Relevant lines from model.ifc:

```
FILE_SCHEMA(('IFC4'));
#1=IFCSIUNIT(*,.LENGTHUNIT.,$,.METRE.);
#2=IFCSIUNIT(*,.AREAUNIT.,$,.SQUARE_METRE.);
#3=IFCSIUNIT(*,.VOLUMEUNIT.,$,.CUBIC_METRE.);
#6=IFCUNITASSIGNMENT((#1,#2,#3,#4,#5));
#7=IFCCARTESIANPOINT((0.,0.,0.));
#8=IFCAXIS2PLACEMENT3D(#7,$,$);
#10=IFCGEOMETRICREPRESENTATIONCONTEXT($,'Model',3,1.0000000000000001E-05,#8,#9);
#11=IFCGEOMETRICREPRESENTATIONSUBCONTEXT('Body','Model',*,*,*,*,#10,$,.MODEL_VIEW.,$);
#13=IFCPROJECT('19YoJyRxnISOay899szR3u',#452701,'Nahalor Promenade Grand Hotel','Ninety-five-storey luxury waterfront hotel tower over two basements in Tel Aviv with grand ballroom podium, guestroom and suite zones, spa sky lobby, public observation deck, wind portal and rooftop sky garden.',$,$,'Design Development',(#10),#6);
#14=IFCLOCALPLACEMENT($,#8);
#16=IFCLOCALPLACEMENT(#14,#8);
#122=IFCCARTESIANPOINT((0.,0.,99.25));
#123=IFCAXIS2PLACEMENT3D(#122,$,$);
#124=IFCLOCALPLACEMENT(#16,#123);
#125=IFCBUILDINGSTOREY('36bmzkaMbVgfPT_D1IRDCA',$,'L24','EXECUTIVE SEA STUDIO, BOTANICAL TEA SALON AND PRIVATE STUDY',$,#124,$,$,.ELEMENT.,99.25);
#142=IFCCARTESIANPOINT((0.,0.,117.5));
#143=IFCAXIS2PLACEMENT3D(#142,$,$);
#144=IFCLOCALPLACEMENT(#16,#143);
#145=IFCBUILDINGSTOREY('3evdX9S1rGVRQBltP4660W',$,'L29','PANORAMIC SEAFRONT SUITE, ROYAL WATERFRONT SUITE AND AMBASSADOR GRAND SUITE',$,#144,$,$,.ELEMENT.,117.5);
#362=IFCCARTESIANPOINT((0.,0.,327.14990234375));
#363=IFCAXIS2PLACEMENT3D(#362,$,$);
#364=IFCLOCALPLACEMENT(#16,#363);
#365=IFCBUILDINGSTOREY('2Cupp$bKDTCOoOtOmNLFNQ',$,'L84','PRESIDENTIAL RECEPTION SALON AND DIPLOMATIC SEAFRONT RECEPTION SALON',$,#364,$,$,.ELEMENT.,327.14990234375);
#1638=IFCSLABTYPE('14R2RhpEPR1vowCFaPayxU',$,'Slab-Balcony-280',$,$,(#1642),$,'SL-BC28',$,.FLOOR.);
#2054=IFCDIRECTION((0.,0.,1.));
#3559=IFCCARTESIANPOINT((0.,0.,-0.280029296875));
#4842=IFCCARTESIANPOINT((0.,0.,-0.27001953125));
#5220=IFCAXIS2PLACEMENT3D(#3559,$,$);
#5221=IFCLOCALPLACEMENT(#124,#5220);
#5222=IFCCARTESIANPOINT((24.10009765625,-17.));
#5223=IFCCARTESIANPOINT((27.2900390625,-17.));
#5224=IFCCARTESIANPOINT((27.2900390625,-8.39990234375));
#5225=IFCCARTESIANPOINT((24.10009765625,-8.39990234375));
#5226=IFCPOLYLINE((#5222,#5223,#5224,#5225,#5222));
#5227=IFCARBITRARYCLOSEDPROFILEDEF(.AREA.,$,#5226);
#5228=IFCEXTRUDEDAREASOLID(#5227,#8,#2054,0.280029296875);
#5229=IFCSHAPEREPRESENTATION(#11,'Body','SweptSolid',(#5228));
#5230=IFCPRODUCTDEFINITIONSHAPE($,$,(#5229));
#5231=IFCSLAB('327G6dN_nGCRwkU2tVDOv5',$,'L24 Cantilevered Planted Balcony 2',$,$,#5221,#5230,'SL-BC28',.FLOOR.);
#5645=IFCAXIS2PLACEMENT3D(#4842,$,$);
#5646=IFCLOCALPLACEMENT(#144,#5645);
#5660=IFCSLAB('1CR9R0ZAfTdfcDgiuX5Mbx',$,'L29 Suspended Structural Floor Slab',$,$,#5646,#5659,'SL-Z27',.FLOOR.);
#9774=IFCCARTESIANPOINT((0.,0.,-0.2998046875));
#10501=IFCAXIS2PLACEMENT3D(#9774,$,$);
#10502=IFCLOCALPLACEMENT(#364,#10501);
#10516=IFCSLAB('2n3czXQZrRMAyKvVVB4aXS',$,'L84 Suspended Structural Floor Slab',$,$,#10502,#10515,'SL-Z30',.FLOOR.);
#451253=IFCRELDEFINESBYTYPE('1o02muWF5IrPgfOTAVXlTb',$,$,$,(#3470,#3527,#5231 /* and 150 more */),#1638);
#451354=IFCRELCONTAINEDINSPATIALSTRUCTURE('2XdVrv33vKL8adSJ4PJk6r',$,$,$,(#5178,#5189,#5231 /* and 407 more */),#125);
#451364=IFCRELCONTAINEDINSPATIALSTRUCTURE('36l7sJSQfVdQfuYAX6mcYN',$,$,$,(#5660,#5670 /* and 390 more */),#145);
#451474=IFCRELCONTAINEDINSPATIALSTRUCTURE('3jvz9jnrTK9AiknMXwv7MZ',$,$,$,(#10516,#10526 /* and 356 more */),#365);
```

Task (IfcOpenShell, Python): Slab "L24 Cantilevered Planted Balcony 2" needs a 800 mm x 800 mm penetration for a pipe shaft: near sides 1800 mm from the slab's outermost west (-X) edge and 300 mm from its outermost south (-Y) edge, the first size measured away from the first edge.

```python
import numpy as np
import ifcopenshell
import ifcopenshell.api.feature
import ifcopenshell.api.geometry
import ifcopenshell.api.root
import ifcopenshell.geom
import ifcopenshell.util.placement
import ifcopenshell.util.representation
import ifcopenshell.util.shape
import ifcopenshell.util.unit

model = ifcopenshell.open("model.ifc")
unit_scale = ifcopenshell.util.unit.calculate_unit_scale(model)
settings = ifcopenshell.geom.settings()


def volume(element):
    """Net volume in cubic metres, openings subtracted."""
    shape = ifcopenshell.geom.create_shape(settings, element)
    return ifcopenshell.util.shape.get_volume(shape.geometry)


slab = model.by_id(5231)
before = volume(slab)

# Extent in the slab's own axes, in metres. The edges named are its -X and -Y sides.
slab_shape = ifcopenshell.geom.create_shape(settings, slab)
vertices = ifcopenshell.util.shape.get_vertices(slab_shape.geometry)
x_min, y_min, bottom = vertices.min(axis=0)
top = vertices[:, 2].max()

opening = ifcopenshell.api.root.create_entity(model, ifc_class="IfcOpeningElement", name="Pipe shaft opening", predefined_type="OPENING")
context = ifcopenshell.util.representation.get_context(model, "Model", "Body", "MODEL_VIEW")
width, depth = 0.8, 0.8
outline = [(0.0, 0.0), (width, 0.0), (width, depth), (0.0, depth), (0.0, 0.0)]
# Overshoot both faces by 50 mm so the cut is clean.
shape = ifcopenshell.api.geometry.add_slab_representation(
    model, context=context, depth=top - bottom + 0.1, polyline=outline
)
ifcopenshell.api.geometry.assign_representation(model, product=opening, representation=shape)

matrix = ifcopenshell.util.placement.get_local_placement(slab.ObjectPlacement)
matrix[:, 3] = matrix @ np.append(np.array([x_min + 1.8, y_min + 0.3, bottom - 0.05]) / unit_scale, 1.0)
ifcopenshell.api.geometry.edit_object_placement(model, product=opening, matrix=matrix, is_si=False)
ifcopenshell.api.feature.add_feature(model, feature=opening, element=slab)

after = volume(slab)

print(f"slab volume {before:.3f} -> {after:.3f} m3")

model.write("model_v2.ifc")
```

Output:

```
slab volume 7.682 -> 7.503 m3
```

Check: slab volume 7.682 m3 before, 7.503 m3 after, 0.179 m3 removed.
